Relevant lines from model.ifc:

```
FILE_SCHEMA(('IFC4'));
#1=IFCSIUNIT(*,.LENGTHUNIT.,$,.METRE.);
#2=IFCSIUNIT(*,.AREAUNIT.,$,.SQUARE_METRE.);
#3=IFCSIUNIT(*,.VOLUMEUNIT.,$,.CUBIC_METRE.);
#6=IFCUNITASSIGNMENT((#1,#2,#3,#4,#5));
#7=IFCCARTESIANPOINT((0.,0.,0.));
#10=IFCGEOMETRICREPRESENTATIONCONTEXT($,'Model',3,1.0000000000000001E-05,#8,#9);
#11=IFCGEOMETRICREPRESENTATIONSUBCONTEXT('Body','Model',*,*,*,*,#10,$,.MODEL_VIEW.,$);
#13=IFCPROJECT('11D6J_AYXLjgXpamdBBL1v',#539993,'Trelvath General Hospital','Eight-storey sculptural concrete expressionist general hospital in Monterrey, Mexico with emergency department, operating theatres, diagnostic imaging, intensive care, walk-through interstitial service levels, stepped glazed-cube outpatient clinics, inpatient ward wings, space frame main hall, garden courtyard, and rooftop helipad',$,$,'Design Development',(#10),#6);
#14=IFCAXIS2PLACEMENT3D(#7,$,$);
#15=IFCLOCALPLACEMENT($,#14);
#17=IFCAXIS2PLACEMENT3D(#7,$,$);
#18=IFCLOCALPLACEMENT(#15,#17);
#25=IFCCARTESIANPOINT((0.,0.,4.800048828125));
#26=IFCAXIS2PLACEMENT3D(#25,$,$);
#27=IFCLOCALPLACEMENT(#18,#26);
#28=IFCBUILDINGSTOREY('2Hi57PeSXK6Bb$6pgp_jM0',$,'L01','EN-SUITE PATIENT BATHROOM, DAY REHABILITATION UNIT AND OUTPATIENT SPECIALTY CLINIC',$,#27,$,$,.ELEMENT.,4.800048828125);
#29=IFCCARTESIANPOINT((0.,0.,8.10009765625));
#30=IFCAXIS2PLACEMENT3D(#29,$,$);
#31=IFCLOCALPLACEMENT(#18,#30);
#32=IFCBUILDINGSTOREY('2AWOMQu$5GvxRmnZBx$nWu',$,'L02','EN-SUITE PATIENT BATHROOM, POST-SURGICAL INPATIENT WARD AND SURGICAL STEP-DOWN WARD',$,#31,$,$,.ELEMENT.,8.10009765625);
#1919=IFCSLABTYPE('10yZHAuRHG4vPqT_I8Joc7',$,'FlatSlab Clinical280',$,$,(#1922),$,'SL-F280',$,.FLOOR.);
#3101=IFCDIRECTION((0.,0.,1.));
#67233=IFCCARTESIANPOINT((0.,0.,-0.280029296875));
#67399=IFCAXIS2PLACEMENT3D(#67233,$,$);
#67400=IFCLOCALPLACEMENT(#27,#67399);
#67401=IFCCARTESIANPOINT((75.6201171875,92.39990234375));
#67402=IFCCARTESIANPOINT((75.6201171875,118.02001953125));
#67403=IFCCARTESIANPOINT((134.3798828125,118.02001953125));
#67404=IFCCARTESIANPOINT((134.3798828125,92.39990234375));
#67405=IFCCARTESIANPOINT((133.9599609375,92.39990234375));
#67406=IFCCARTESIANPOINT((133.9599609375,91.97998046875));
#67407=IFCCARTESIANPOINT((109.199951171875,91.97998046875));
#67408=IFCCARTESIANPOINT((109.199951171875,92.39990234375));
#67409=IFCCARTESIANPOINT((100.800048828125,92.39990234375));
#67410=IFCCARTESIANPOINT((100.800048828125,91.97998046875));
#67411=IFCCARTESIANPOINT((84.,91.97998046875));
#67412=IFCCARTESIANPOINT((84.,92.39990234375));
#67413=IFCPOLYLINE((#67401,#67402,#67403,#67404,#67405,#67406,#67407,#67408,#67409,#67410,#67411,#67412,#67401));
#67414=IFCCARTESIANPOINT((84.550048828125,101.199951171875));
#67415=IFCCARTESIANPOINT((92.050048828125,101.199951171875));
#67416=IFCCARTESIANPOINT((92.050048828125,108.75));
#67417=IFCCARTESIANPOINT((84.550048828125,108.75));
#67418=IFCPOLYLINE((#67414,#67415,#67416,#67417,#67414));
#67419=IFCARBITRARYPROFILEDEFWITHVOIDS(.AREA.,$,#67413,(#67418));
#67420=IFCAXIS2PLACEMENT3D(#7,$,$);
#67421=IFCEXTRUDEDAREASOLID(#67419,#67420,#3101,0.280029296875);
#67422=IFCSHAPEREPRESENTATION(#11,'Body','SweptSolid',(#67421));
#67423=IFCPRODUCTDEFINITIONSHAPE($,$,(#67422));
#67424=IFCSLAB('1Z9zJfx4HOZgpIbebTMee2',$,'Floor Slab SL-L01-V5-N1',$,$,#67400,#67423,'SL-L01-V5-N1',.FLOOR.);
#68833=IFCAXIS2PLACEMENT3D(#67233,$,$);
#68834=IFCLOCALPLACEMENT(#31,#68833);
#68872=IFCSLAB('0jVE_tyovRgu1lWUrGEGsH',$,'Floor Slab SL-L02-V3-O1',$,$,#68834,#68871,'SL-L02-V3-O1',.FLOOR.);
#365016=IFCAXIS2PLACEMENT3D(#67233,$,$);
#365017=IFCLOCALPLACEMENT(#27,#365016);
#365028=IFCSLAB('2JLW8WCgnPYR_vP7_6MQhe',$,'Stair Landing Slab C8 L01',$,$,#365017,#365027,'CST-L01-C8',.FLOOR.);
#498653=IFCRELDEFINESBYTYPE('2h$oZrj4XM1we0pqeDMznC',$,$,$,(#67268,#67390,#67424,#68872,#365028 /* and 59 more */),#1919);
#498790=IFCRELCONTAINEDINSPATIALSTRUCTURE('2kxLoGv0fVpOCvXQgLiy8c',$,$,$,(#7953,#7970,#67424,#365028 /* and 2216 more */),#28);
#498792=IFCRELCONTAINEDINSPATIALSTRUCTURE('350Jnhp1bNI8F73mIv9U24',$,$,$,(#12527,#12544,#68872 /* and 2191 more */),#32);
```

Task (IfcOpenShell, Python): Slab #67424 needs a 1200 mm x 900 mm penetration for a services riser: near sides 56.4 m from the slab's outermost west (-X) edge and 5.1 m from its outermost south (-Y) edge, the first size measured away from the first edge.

```python
import numpy as np
import ifcopenshell
import ifcopenshell.api.feature
import ifcopenshell.api.geometry
import ifcopenshell.api.root
import ifcopenshell.geom
import ifcopenshell.util.placement
import ifcopenshell.util.representation
import ifcopenshell.util.shape
import ifcopenshell.util.unit

model = ifcopenshell.open("model.ifc")
unit_scale = ifcopenshell.util.unit.calculate_unit_scale(model)
settings = ifcopenshell.geom.settings()


def volume(element):
    """Net volume in cubic metres, openings subtracted."""
    shape = ifcopenshell.geom.create_shape(settings, element)
    return ifcopenshell.util.shape.get_volume(shape.geometry)


slab = model.by_guid("1Z9zJfx4HOZgpIbebTMee2")
before = volume(slab)

# Extent in the slab's own axes, in metres. The edges named are its -X and -Y sides.
slab_shape = ifcopenshell.geom.create_shape(settings, slab)
vertices = ifcopenshell.util.shape.get_vertices(slab_shape.geometry)
x_min, y_min, bottom = vertices.min(axis=0)
top = vertices[:, 2].max()

opening = ifcopenshell.api.root.create_entity(model, ifc_class="IfcOpeningElement", name="Services riser opening", predefined_type="OPENING")
context = ifcopenshell.util.representation.get_context(model, "Model", "Body", "MODEL_VIEW")
width, depth = 1.2, 0.9
outline = [(0.0, 0.0), (width, 0.0), (width, depth), (0.0, depth), (0.0, 0.0)]
# Overshoot both faces by 50 mm so the cut is clean.
shape = ifcopenshell.api.geometry.add_slab_representation(
    model, context=context, depth=top - bottom + 0.1, polyline=outline
)
ifcopenshell.api.geometry.assign_representation(model, product=opening, representation=shape)

matrix = ifcopenshell.util.placement.get_local_placement(slab.ObjectPlacement)
matrix[:, 3] = matrix @ np.append(np.array([x_min + 56.4, y_min + 5.1, bottom - 0.05]) / unit_scale, 1.0)
ifcopenshell.api.geometry.edit_object_placement(model, product=opening, matrix=matrix, is_si=False)
ifcopenshell.api.feature.add_feature(model, feature=opening, element=slab)

after = volume(slab)

print(f"slab volume {before:.3f} -> {after:.3f} m3")

model.write("model-out.ifc")
```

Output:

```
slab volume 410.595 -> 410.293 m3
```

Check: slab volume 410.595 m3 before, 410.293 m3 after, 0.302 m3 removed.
